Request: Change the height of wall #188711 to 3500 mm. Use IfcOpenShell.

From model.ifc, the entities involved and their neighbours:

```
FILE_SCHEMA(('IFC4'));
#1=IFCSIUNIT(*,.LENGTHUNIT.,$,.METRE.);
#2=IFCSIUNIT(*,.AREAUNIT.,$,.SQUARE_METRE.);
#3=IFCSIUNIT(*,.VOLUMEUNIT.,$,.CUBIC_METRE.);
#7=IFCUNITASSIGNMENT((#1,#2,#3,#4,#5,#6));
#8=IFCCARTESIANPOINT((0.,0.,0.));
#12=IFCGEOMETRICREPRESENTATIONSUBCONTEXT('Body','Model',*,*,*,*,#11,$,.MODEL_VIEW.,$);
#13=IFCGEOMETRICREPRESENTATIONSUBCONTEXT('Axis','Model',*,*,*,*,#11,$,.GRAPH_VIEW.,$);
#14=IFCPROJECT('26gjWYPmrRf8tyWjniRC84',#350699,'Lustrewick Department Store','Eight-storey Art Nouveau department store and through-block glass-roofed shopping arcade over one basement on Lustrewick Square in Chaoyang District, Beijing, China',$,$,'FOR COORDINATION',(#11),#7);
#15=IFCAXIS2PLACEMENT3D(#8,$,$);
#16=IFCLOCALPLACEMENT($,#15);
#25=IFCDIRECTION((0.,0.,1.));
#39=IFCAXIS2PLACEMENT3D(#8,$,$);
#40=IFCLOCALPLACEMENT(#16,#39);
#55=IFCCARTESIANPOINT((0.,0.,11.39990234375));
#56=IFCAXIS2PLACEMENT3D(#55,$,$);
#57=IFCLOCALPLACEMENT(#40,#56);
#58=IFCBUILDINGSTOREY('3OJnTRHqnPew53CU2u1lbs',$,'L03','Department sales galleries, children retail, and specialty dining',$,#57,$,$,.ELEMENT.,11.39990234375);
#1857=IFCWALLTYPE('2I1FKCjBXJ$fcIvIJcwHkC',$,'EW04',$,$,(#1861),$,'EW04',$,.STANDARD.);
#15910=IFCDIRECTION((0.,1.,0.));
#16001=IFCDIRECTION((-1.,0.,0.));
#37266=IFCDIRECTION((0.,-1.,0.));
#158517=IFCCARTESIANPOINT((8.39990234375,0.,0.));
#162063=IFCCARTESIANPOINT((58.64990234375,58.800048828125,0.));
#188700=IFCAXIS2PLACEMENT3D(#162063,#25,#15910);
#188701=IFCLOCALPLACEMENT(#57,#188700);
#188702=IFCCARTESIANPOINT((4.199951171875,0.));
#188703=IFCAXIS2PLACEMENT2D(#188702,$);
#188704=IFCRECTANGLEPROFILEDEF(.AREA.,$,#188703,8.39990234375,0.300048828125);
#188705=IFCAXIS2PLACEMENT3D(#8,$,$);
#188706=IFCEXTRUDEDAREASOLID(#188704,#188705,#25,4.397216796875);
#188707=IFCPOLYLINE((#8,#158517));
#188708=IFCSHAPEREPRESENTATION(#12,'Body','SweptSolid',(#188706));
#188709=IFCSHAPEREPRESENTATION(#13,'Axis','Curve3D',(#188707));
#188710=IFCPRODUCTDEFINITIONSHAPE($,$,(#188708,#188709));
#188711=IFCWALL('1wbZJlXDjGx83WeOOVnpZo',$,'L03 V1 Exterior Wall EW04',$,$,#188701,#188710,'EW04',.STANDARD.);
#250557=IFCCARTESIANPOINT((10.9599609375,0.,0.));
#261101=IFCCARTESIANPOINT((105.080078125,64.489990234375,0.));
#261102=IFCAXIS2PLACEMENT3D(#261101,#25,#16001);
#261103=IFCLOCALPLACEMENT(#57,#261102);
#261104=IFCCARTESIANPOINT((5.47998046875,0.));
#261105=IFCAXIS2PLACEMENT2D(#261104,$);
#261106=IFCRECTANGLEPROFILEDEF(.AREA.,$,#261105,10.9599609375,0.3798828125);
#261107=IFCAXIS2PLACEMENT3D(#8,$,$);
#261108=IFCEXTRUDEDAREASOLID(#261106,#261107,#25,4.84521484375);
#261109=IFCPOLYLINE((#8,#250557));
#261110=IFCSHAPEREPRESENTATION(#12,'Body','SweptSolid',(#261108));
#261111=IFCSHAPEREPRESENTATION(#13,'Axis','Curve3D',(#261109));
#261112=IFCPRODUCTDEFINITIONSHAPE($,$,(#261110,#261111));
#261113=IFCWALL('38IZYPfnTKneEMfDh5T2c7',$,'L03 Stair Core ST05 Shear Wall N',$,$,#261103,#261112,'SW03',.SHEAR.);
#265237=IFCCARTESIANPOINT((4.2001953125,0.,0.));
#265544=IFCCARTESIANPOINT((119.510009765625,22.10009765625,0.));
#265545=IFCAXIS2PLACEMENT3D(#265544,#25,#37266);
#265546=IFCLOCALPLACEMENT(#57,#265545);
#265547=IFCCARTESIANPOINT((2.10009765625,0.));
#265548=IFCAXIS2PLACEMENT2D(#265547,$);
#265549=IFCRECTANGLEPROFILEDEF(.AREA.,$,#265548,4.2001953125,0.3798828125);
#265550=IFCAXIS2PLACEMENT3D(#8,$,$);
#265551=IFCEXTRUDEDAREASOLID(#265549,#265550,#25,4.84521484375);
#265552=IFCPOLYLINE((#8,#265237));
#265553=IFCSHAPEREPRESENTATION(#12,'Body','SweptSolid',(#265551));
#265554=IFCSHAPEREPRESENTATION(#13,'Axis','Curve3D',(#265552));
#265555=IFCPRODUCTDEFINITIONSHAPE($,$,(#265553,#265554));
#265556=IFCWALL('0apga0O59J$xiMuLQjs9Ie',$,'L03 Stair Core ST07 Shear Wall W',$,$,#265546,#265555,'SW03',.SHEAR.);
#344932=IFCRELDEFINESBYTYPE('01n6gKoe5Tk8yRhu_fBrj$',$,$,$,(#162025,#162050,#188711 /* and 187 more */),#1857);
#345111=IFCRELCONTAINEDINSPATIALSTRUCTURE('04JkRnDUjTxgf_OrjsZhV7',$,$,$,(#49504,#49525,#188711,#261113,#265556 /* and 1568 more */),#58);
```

```python
import ifcopenshell
import ifcopenshell.geom
import ifcopenshell.util.representation
import ifcopenshell.util.shape
import ifcopenshell.util.unit

model = ifcopenshell.open("model.ifc")
unit_scale = ifcopenshell.util.unit.calculate_unit_scale(model)
settings = ifcopenshell.geom.settings()


def volume(element):
    """Net volume in cubic metres, openings subtracted."""
    shape = ifcopenshell.geom.create_shape(settings, element)
    return ifcopenshell.util.shape.get_volume(shape.geometry)


wall = model.by_guid("1wbZJlXDjGx83WeOOVnpZo")
before = volume(wall)

body = ifcopenshell.util.representation.get_representation(wall, "Model", "Body")
solid = body.Items[0]
old_height = solid.Depth
solid.Depth = 3.5 / unit_scale
after = volume(wall)

print(f"height {old_height:g} -> {solid.Depth:g}, volume {before:.3f} -> {after:.3f} m3")

model.write("model_updated.ifc")
```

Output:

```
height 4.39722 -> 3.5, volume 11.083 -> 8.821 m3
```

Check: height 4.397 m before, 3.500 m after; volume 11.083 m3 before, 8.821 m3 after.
